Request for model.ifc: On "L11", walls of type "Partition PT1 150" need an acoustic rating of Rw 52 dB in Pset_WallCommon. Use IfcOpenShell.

First a look at what the model holds.

```python
import ifcopenshell
import ifcopenshell.util.element

model = ifcopenshell.open("model.ifc")
print(model.schema)
storey = next(s for s in model.by_type("IfcBuildingStorey") if s.Name == "L11")
walls = [e for e in ifcopenshell.util.element.get_decomposition(storey) if e.is_a("IfcWall")]
seen = {}
for e in walls:
    element_type = ifcopenshell.util.element.get_type(e)
    key = (element_type.Name if element_type != e and element_type else None, ifcopenshell.util.element.get_pset(e, "Pset_WallCommon", "AcousticRating"))
    seen[key] = seen.get(key, 0) + 1
for (name, value), count in sorted(seen.items(), key=str):
    print(count, "x", name, "|", value)
```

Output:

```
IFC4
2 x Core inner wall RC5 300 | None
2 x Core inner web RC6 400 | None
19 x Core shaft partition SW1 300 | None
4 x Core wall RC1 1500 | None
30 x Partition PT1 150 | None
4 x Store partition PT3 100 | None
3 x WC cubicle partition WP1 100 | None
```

```python
import ifcopenshell
import ifcopenshell.api.pset
import ifcopenshell.util.element

model = ifcopenshell.open("model.ifc")

storey = next(s for s in model.by_type("IfcBuildingStorey") if s.Name == "L11")
walls = [e for e in ifcopenshell.util.element.get_decomposition(storey) if e.is_a("IfcWall")]

count = 0
for e in walls:
    element_type = ifcopenshell.util.element.get_type(e)
    if element_type in (None, e) or element_type.Name != "Partition PT1 150":
        continue
    # add_pset returns the element's existing set when there is one.
    pset = ifcopenshell.api.pset.add_pset(model, product=e, name="Pset_WallCommon")
    ifcopenshell.api.pset.edit_pset(model, pset=pset, properties={"AcousticRating": "Rw 52 dB"})
    count += 1

print(count, "walls updated")

model.write("model-out.ifc")
```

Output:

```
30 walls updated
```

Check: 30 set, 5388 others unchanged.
